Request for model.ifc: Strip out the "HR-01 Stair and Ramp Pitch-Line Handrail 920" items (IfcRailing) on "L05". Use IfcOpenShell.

First a look at what the model holds.

```python
import ifcopenshell
import ifcopenshell.util.element

model = ifcopenshell.open("model.ifc")
print(model.schema)
storey = next(s for s in model.by_type("IfcBuildingStorey") if s.Name == "L05")
railings = [e for e in ifcopenshell.util.element.get_decomposition(storey) if e.is_a("IfcRailing")]
seen = {}
for e in railings:
    element_type = ifcopenshell.util.element.get_type(e)
    name = element_type.Name if element_type not in (None, e) else None
    seen[name] = seen.get(name, 0) + 1
for name, count in sorted(seen.items(), key=str):
    print(count, "x", name)
```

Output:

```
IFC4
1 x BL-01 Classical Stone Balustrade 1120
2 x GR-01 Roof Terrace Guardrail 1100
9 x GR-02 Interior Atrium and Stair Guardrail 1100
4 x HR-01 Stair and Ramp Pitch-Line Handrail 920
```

```python
import ifcopenshell
import ifcopenshell.api.root
import ifcopenshell.util.element

model = ifcopenshell.open("model.ifc")

storey = next(s for s in model.by_type("IfcBuildingStorey") if s.Name == "L05")
railings = [e for e in ifcopenshell.util.element.get_decomposition(storey) if e.is_a("IfcRailing")]
targets = [e for e in railings if (t := ifcopenshell.util.element.get_type(e)) not in (None, e) and t.Name == "HR-01 Stair and Ramp Pitch-Line Handrail 920"]

for e in targets:
    ifcopenshell.api.root.remove_product(model, product=e)
print(len(targets), "removed")

model.write("model_rev.ifc")
```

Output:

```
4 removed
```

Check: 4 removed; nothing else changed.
